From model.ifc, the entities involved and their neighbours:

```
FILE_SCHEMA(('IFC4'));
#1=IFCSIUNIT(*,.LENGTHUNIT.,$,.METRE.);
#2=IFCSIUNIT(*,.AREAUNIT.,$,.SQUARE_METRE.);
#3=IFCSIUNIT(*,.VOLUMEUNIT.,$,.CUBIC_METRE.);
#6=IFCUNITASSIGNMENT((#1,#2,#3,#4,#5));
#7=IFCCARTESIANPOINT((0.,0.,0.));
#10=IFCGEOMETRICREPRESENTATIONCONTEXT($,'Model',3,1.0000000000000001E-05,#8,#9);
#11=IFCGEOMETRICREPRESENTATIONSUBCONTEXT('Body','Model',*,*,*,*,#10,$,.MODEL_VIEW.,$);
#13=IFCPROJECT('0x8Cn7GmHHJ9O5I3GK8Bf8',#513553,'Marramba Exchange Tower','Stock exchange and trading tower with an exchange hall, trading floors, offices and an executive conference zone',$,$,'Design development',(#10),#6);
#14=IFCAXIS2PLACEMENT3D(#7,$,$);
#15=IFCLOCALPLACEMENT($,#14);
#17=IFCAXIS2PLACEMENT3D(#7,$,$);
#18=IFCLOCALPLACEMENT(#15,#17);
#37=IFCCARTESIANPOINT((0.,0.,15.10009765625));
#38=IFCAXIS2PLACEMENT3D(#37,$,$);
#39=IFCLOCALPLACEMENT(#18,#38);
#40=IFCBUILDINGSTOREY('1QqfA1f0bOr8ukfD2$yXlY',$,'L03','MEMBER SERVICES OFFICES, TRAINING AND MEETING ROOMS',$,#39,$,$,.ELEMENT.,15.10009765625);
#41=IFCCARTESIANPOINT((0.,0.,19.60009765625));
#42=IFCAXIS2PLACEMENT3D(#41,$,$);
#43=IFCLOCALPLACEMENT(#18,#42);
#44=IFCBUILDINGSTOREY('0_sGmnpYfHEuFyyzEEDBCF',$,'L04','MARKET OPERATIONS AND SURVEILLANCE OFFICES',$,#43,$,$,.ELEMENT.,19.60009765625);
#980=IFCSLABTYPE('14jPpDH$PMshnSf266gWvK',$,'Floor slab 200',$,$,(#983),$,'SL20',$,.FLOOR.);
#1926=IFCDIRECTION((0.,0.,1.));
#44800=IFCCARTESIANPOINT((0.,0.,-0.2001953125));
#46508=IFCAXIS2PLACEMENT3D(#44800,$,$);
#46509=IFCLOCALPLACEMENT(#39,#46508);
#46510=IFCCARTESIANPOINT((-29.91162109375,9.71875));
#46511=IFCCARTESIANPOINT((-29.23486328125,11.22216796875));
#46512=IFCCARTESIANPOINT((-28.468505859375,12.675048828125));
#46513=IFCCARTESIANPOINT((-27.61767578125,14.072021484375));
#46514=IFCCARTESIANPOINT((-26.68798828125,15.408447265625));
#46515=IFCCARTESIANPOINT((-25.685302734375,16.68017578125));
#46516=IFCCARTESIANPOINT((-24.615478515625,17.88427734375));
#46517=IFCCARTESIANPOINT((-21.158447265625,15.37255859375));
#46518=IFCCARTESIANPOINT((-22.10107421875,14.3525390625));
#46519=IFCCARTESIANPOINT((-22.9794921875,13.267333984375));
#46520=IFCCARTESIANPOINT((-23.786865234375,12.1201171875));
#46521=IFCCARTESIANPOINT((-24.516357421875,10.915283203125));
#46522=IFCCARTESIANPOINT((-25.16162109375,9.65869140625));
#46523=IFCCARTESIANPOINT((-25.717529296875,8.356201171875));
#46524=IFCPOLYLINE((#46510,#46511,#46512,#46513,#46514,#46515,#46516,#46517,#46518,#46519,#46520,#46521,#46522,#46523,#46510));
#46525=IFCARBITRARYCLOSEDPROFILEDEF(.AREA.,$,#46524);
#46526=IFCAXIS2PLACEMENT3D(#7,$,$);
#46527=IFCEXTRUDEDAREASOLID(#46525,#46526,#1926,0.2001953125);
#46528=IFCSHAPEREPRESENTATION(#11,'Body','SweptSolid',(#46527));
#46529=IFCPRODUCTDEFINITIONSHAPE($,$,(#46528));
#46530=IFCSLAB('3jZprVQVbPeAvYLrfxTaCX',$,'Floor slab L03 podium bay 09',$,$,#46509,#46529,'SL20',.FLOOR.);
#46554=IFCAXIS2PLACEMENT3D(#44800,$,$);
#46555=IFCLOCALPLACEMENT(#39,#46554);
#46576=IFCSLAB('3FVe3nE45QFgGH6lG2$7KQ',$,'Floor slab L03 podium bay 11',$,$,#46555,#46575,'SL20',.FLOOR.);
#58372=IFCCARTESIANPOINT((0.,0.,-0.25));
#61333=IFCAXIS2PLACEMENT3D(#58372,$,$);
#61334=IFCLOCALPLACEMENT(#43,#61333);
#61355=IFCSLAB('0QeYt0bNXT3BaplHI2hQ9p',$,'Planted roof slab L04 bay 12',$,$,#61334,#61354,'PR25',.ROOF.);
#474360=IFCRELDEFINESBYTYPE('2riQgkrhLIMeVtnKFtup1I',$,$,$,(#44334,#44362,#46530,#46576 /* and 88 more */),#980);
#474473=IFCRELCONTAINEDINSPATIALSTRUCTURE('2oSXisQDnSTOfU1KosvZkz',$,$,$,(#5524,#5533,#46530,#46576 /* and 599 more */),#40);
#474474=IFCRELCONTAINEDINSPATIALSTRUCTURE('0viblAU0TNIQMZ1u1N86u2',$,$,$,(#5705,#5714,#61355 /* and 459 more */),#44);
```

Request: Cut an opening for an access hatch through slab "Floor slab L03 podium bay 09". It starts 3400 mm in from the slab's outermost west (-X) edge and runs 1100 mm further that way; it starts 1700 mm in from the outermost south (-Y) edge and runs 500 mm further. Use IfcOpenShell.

```python
import numpy as np
import ifcopenshell
import ifcopenshell.api.feature
import ifcopenshell.api.geometry
import ifcopenshell.api.root
import ifcopenshell.geom
import ifcopenshell.util.placement
import ifcopenshell.util.representation
import ifcopenshell.util.shape
import ifcopenshell.util.unit

model = ifcopenshell.open("model.ifc")
unit_scale = ifcopenshell.util.unit.calculate_unit_scale(model)
settings = ifcopenshell.geom.settings()


def volume(element):
    """Net volume in cubic metres, openings subtracted."""
    shape = ifcopenshell.geom.create_shape(settings, element)
    return ifcopenshell.util.shape.get_volume(shape.geometry)


slab = model.by_guid("3jZprVQVbPeAvYLrfxTaCX")
before = volume(slab)

# Extent in the slab's own axes, in metres. The edges named are its -X and -Y sides.
slab_shape = ifcopenshell.geom.create_shape(settings, slab)
vertices = ifcopenshell.util.shape.get_vertices(slab_shape.geometry)
x_min, y_min, bottom = vertices.min(axis=0)
top = vertices[:, 2].max()

opening = ifcopenshell.api.root.create_entity(model, ifc_class="IfcOpeningElement", name="Access hatch opening", predefined_type="OPENING")
context = ifcopenshell.util.representation.get_context(model, "Model", "Body", "MODEL_VIEW")
width, depth = 1.1, 0.5
outline = [(0.0, 0.0), (width, 0.0), (width, depth), (0.0, depth), (0.0, 0.0)]
# Overshoot both faces by 50 mm so the cut is clean.
shape = ifcopenshell.api.geometry.add_slab_representation(
    model, context=context, depth=top - bottom + 0.1, polyline=outline
)
ifcopenshell.api.geometry.assign_representation(model, product=opening, representation=shape)

matrix = ifcopenshell.util.placement.get_local_placement(slab.ObjectPlacement)
matrix[:, 3] = matrix @ np.append(np.array([x_min + 3.4, y_min + 1.7, bottom - 0.05]) / unit_scale, 1.0)
ifcopenshell.api.geometry.edit_object_placement(model, product=opening, matrix=matrix, is_si=False)
ifcopenshell.api.feature.add_feature(model, feature=opening, element=slab)

after = volume(slab)

print(f"slab volume {before:.3f} -> {after:.3f} m3")

model.write("model_rev.ifc")
```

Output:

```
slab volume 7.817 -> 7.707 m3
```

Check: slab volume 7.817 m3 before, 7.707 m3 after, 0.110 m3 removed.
